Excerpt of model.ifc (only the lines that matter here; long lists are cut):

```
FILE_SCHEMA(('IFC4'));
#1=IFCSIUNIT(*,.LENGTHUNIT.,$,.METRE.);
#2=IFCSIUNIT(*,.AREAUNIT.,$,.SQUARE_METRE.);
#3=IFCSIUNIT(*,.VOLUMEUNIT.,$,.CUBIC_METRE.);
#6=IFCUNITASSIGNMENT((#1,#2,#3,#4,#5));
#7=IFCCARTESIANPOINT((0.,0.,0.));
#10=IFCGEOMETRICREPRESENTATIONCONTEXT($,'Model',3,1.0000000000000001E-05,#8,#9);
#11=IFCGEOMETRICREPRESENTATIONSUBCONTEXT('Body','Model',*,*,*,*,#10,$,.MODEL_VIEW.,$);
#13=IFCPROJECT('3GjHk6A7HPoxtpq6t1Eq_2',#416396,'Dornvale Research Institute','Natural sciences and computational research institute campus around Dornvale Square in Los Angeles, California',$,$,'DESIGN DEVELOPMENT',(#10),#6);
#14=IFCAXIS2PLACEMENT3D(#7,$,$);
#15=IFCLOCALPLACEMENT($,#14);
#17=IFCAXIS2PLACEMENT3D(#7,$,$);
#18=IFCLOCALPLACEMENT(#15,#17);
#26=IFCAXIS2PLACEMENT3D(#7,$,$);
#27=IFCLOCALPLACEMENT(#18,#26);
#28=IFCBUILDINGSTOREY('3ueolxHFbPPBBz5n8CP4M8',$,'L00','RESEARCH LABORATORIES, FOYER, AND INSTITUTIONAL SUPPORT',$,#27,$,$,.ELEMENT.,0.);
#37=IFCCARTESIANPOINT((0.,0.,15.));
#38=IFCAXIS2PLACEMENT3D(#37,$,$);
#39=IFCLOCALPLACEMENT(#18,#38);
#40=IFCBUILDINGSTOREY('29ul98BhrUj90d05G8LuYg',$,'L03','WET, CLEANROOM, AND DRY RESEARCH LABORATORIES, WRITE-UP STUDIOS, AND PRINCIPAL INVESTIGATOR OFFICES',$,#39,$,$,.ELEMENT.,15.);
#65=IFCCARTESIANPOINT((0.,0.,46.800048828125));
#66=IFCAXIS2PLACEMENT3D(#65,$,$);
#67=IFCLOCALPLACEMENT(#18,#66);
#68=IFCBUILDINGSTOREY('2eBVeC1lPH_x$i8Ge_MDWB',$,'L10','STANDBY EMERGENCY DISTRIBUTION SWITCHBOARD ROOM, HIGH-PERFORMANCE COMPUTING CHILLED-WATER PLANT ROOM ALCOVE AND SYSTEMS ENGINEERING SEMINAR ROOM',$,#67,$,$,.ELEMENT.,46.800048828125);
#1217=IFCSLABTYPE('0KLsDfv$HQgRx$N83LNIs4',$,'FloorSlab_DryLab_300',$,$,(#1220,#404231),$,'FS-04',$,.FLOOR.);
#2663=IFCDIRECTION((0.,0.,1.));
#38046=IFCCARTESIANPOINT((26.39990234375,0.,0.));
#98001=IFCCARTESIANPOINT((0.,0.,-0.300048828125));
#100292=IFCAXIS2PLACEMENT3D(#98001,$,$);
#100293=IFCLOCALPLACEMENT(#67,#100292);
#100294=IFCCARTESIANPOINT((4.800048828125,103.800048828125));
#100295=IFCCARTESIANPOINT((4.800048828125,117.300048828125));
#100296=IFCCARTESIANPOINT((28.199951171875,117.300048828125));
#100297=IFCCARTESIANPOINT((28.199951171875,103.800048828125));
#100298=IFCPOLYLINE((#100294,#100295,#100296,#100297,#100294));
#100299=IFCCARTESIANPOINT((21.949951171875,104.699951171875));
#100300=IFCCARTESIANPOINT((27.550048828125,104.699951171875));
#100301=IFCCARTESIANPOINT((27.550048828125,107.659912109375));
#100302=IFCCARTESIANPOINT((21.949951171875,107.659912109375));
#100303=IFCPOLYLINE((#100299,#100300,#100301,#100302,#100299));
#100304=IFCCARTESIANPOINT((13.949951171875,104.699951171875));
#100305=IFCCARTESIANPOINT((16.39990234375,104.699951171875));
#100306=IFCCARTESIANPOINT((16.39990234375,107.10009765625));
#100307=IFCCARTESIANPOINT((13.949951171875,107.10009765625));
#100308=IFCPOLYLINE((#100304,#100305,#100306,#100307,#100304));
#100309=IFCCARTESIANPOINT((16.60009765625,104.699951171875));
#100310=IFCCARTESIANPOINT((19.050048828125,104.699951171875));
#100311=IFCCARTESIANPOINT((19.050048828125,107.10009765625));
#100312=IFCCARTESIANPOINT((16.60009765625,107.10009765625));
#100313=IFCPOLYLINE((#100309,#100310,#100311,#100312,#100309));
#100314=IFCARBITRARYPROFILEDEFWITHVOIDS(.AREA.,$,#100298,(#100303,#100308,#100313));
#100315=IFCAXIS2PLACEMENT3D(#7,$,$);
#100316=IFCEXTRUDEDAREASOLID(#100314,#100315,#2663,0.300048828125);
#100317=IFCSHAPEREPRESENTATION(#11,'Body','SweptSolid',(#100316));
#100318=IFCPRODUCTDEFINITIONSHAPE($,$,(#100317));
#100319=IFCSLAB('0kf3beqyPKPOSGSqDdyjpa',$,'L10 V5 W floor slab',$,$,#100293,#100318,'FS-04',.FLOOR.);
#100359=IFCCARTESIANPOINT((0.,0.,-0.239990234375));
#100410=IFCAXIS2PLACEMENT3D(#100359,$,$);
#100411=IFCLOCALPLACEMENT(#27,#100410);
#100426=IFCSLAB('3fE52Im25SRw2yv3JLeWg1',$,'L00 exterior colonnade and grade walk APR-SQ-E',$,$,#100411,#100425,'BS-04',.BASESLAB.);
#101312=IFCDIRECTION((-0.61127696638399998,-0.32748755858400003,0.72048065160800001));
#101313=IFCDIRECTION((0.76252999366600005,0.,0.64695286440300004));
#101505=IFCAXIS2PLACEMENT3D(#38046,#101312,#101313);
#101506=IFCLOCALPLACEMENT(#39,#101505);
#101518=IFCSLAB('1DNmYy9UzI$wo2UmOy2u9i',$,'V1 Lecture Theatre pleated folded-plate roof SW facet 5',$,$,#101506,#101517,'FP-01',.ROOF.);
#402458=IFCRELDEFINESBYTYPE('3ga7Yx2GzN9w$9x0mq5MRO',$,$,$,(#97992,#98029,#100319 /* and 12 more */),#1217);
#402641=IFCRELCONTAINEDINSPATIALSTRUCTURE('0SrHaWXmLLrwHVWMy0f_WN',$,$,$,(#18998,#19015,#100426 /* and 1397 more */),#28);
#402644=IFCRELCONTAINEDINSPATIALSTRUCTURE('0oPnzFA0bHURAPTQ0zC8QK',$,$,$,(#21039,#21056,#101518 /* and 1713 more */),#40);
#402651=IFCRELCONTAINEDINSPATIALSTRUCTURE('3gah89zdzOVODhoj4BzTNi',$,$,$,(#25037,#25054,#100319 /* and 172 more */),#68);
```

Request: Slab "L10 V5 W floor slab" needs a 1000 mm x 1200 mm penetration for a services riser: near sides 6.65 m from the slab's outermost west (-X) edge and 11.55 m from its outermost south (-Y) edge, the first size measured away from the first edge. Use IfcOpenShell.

```python
import numpy as np
import ifcopenshell
import ifcopenshell.api.feature
import ifcopenshell.api.geometry
import ifcopenshell.api.root
import ifcopenshell.geom
import ifcopenshell.util.placement
import ifcopenshell.util.representation
import ifcopenshell.util.shape
import ifcopenshell.util.unit

model = ifcopenshell.open("model.ifc")
unit_scale = ifcopenshell.util.unit.calculate_unit_scale(model)
settings = ifcopenshell.geom.settings()


def volume(element):
    """Net volume in cubic metres, openings subtracted."""
    shape = ifcopenshell.geom.create_shape(settings, element)
    return ifcopenshell.util.shape.get_volume(shape.geometry)


slab = model.by_id(100319)
before = volume(slab)

# Extent in the slab's own axes, in metres. The edges named are its -X and -Y sides.
slab_shape = ifcopenshell.geom.create_shape(settings, slab)
vertices = ifcopenshell.util.shape.get_vertices(slab_shape.geometry)
x_min, y_min, bottom = vertices.min(axis=0)
top = vertices[:, 2].max()

opening = ifcopenshell.api.root.create_entity(model, ifc_class="IfcOpeningElement", name="Services riser opening", predefined_type="OPENING")
context = ifcopenshell.util.representation.get_context(model, "Model", "Body", "MODEL_VIEW")
width, depth = 1, 1.2
outline = [(0.0, 0.0), (width, 0.0), (width, depth), (0.0, depth), (0.0, 0.0)]
# Overshoot both faces by 50 mm so the cut is clean.
shape = ifcopenshell.api.geometry.add_slab_representation(
    model, context=context, depth=top - bottom + 0.1, polyline=outline
)
ifcopenshell.api.geometry.assign_representation(model, product=opening, representation=shape)

matrix = ifcopenshell.util.placement.get_local_placement(slab.ObjectPlacement)
matrix[:, 3] = matrix @ np.append(np.array([x_min + 6.65, y_min + 11.55, bottom - 0.05]) / unit_scale, 1.0)
ifcopenshell.api.geometry.edit_object_placement(model, product=opening, matrix=matrix, is_si=False)
ifcopenshell.api.feature.add_feature(model, feature=opening, element=slab)

after = volume(slab)

print(f"slab volume {before:.3f} -> {after:.3f} m3")

model.write("model_updated.ifc")
```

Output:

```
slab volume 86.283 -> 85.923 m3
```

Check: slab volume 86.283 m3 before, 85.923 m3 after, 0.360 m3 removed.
